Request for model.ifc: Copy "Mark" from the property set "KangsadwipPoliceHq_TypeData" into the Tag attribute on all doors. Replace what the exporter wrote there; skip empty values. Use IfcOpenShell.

First a look at what the model holds.

```python
import ifcopenshell
import ifcopenshell.util.element

model = ifcopenshell.open("model.ifc")
print(model.schema)
doors = model.by_type("IfcDoor")
print(len(doors), "doors")
for e in doors[:8]:
    source = ifcopenshell.util.element.get_pset(e, "KangsadwipPoliceHq_TypeData", "Mark")
    target = e.Tag
    print(e.id(), repr(source), repr(target), sep=" | ")
```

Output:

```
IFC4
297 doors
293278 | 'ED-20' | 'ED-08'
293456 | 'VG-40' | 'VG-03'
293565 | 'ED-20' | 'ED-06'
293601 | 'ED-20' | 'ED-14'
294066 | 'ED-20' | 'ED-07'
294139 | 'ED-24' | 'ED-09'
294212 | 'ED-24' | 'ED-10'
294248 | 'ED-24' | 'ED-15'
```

```python
import ifcopenshell
import ifcopenshell.util.element

model = ifcopenshell.open("model.ifc")

count = 0
for e in model.by_type("IfcDoor"):
    value = ifcopenshell.util.element.get_pset(e, "KangsadwipPoliceHq_TypeData", "Mark")
    current = e.Tag
    if not value or not value.strip() or current == value:
        continue
    e.Tag = value
    count += 1

print(count, "doors updated")

model.write("model-out.ifc")
```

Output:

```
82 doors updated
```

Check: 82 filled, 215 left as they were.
